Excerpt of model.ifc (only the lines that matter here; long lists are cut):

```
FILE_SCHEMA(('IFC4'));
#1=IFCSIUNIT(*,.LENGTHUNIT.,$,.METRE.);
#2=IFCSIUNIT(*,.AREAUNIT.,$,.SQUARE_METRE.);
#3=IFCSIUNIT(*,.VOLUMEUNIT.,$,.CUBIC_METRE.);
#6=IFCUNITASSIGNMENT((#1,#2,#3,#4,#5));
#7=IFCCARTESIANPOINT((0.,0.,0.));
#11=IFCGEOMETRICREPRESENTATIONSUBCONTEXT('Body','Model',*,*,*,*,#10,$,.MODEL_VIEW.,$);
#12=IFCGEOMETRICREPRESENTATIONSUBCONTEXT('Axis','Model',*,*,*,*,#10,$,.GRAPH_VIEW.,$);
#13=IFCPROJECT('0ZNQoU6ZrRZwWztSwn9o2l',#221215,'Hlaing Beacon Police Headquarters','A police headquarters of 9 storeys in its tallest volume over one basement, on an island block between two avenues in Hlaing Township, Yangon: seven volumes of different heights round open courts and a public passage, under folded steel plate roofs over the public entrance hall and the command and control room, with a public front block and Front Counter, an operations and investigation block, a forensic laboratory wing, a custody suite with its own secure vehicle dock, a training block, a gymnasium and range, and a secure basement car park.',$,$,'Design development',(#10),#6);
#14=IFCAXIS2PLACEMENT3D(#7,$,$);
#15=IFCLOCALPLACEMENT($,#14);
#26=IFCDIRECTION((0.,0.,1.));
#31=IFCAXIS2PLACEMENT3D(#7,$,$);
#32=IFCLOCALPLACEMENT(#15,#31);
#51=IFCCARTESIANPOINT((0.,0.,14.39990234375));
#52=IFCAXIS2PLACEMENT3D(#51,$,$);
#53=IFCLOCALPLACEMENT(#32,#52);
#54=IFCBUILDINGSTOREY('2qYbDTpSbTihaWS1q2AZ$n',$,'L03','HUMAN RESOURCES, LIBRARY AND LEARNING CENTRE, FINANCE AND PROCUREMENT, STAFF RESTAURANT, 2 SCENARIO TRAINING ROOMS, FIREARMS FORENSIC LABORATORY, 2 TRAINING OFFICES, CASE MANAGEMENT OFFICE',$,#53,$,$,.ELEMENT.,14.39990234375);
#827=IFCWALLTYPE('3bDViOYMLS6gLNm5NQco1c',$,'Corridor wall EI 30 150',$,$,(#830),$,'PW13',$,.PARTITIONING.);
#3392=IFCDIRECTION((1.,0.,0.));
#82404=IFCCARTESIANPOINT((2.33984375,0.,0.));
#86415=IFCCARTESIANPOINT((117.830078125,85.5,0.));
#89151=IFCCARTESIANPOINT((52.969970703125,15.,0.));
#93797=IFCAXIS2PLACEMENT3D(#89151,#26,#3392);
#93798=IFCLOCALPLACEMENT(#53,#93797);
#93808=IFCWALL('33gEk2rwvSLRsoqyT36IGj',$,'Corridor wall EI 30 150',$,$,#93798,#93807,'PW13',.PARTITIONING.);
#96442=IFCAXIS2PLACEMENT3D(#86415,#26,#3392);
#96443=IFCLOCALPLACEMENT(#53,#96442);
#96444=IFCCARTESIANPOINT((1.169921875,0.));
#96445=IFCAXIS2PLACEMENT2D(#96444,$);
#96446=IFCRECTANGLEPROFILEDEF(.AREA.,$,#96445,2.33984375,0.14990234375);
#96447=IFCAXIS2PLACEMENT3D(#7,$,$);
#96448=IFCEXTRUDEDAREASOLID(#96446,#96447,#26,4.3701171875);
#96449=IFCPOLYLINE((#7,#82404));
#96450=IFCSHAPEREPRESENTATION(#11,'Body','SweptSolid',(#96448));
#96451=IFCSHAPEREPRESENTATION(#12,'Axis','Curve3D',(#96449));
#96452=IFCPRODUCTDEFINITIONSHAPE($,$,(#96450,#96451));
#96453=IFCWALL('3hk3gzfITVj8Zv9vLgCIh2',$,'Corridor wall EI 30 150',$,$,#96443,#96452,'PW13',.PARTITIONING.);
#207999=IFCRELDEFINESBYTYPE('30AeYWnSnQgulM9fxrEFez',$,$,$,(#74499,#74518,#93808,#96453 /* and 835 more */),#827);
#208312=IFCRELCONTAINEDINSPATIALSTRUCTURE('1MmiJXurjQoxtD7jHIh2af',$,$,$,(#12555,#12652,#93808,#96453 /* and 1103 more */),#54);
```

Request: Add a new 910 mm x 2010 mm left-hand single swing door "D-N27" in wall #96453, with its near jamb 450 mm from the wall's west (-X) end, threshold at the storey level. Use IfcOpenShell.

```python
import numpy as np
import ifcopenshell
import ifcopenshell.api.feature
import ifcopenshell.api.geometry
import ifcopenshell.api.root
import ifcopenshell.api.spatial
import ifcopenshell.geom
import ifcopenshell.util.element
import ifcopenshell.util.placement
import ifcopenshell.util.representation
import ifcopenshell.util.shape
import ifcopenshell.util.unit

model = ifcopenshell.open("model.ifc")
unit_scale = ifcopenshell.util.unit.calculate_unit_scale(model)
settings = ifcopenshell.geom.settings()


def volume(element):
    """Net volume in cubic metres, openings subtracted."""
    shape = ifcopenshell.geom.create_shape(settings, element)
    return ifcopenshell.util.shape.get_volume(shape.geometry)


wall = model.by_guid("3hk3gzfITVj8Zv9vLgCIh2")
storey = ifcopenshell.util.element.get_container(wall, ifc_class="IfcBuildingStorey")
context = ifcopenshell.util.representation.get_context(model, "Model", "Body", "MODEL_VIEW")
before = volume(wall)

width, height, from_end, sill = 0.91, 2.01, 0.45, 0.0  # metres

# The wall runs along its own X axis, and the end named is its -X end.
wall_shape = ifcopenshell.geom.create_shape(settings, wall)
x, y, z = ifcopenshell.util.shape.get_vertices(wall_shape.geometry).T
start = x.min() + from_end
face, thickness = float(y.min()), float(y.max() - y.min())
wall_matrix = ifcopenshell.util.placement.get_local_placement(wall.ObjectPlacement)
level = ifcopenshell.util.placement.get_local_placement(storey.ObjectPlacement)[2, 3]


def in_wall(x, y):
    """Placement at x, y metres in the wall's axes, at sill height."""
    matrix = wall_matrix.copy()
    matrix[:, 3] = wall_matrix @ np.array([x / unit_scale, y / unit_scale, 0.0, 1.0])
    matrix[2, 3] = level + sill / unit_scale
    return matrix


# Opening: a box that overshoots both wall faces by 50 mm.
opening = ifcopenshell.api.root.create_entity(model, ifc_class="IfcOpeningElement", predefined_type="OPENING")
box = ifcopenshell.api.geometry.add_wall_representation(
    model, context=context, length=width, height=height, thickness=thickness + 0.1
)
ifcopenshell.api.geometry.assign_representation(model, product=opening, representation=box)
ifcopenshell.api.geometry.edit_object_placement(model, product=opening, matrix=in_wall(start, face - 0.05), is_si=False)
ifcopenshell.api.feature.add_feature(model, feature=opening, element=wall)

door = ifcopenshell.api.root.create_entity(model, ifc_class="IfcDoor", name="D-N27", predefined_type="DOOR")
door.OverallWidth, door.OverallHeight = width / unit_scale, height / unit_scale
door.OperationType = "SINGLE_SWING_LEFT"
body = ifcopenshell.api.geometry.add_door_representation(
    model,
    context=context,
    overall_width=door.OverallWidth,
    overall_height=door.OverallHeight,
    operation_type="SINGLE_SWING_LEFT",
    lining_properties={"LiningDepth": thickness / unit_scale, "ThresholdDepth": thickness / unit_scale},
)
ifcopenshell.api.geometry.assign_representation(model, product=door, representation=body)
ifcopenshell.api.spatial.assign_container(model, products=[door], relating_structure=storey)
ifcopenshell.api.feature.add_filling(model, opening=opening, element=door)

# The lining spans the wall, so the door starts at the wall face.
ifcopenshell.api.geometry.edit_object_placement(model, product=door, matrix=in_wall(start, face), is_si=False)

after = volume(wall)

print(f"wall volume {before:.3f} -> {after:.3f} m3")

model.write("model-out.ifc")
```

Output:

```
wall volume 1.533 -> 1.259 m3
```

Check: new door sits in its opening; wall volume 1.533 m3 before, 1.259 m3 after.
